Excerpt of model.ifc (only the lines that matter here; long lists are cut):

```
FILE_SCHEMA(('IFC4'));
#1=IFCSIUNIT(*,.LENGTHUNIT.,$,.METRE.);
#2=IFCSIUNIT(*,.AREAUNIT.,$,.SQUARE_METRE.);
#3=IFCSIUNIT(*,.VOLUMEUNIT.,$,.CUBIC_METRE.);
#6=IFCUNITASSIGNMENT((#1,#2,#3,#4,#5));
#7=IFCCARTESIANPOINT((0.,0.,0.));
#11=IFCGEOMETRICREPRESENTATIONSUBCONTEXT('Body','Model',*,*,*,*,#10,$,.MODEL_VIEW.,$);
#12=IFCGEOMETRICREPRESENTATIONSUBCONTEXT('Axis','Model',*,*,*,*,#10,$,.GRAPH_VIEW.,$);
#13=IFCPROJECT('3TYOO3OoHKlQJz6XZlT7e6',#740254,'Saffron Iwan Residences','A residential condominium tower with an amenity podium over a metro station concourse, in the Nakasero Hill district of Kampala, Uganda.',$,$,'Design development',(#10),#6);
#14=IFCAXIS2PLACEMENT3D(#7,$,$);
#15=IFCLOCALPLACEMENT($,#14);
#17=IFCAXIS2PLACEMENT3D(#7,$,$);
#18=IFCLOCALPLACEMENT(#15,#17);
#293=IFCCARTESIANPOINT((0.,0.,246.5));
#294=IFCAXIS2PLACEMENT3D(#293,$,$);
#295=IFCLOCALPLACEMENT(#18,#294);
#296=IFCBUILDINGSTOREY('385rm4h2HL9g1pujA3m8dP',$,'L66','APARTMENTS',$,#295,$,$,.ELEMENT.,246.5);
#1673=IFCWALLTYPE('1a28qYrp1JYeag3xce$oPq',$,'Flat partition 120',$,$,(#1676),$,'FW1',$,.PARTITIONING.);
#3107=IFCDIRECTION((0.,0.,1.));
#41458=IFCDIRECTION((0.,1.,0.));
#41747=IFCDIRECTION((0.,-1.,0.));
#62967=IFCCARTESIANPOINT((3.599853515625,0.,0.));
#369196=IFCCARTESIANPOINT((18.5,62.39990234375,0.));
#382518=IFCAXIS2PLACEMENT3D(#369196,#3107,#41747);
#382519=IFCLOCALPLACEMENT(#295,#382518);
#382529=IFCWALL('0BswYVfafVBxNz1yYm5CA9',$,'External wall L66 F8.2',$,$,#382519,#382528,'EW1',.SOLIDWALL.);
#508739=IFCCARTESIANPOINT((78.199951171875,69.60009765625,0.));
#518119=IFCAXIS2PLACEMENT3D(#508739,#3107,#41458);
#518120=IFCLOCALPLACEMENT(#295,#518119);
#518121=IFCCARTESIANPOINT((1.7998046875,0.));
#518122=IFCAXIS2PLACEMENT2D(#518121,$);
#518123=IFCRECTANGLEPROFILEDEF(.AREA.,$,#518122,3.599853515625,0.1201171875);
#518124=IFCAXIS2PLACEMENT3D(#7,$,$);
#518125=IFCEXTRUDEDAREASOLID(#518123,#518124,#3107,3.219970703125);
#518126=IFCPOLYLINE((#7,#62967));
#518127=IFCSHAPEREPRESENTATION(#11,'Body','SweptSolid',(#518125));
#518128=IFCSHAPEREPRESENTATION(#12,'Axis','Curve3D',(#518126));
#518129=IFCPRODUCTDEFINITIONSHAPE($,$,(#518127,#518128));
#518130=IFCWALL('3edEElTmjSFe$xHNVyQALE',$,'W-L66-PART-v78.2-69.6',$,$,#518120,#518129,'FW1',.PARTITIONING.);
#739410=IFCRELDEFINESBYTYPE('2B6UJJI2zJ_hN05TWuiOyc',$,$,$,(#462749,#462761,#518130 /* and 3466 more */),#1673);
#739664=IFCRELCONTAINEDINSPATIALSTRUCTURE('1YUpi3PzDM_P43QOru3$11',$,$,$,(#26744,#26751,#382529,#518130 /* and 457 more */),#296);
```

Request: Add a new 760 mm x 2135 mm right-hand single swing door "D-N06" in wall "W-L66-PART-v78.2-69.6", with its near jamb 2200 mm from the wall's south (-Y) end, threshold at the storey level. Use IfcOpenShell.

```python
import numpy as np
import ifcopenshell
import ifcopenshell.api.feature
import ifcopenshell.api.geometry
import ifcopenshell.api.root
import ifcopenshell.api.spatial
import ifcopenshell.geom
import ifcopenshell.util.element
import ifcopenshell.util.placement
import ifcopenshell.util.representation
import ifcopenshell.util.shape
import ifcopenshell.util.unit

model = ifcopenshell.open("model.ifc")
unit_scale = ifcopenshell.util.unit.calculate_unit_scale(model)
settings = ifcopenshell.geom.settings()


def volume(element):
    """Net volume in cubic metres, openings subtracted."""
    shape = ifcopenshell.geom.create_shape(settings, element)
    return ifcopenshell.util.shape.get_volume(shape.geometry)


wall = model.by_guid("3edEElTmjSFe$xHNVyQALE")
storey = ifcopenshell.util.element.get_container(wall, ifc_class="IfcBuildingStorey")
context = ifcopenshell.util.representation.get_context(model, "Model", "Body", "MODEL_VIEW")
before = volume(wall)

width, height, from_end, sill = 0.76, 2.135, 2.2, 0.0  # metres

# The wall runs along its own X axis, and the end named is its -X end.
wall_shape = ifcopenshell.geom.create_shape(settings, wall)
x, y, z = ifcopenshell.util.shape.get_vertices(wall_shape.geometry).T
start = x.min() + from_end
face, thickness = float(y.min()), float(y.max() - y.min())
wall_matrix = ifcopenshell.util.placement.get_local_placement(wall.ObjectPlacement)
level = ifcopenshell.util.placement.get_local_placement(storey.ObjectPlacement)[2, 3]


def in_wall(x, y):
    """Placement at x, y metres in the wall's axes, at sill height."""
    matrix = wall_matrix.copy()
    matrix[:, 3] = wall_matrix @ np.array([x / unit_scale, y / unit_scale, 0.0, 1.0])
    matrix[2, 3] = level + sill / unit_scale
    return matrix


# Opening: a box that overshoots both wall faces by 50 mm.
opening = ifcopenshell.api.root.create_entity(model, ifc_class="IfcOpeningElement", predefined_type="OPENING")
box = ifcopenshell.api.geometry.add_wall_representation(
    model, context=context, length=width, height=height, thickness=thickness + 0.1
)
ifcopenshell.api.geometry.assign_representation(model, product=opening, representation=box)
ifcopenshell.api.geometry.edit_object_placement(model, product=opening, matrix=in_wall(start, face - 0.05), is_si=False)
ifcopenshell.api.feature.add_feature(model, feature=opening, element=wall)

door = ifcopenshell.api.root.create_entity(model, ifc_class="IfcDoor", name="D-N06", predefined_type="DOOR")
door.OverallWidth, door.OverallHeight = width / unit_scale, height / unit_scale
door.OperationType = "SINGLE_SWING_RIGHT"
body = ifcopenshell.api.geometry.add_door_representation(
    model,
    context=context,
    overall_width=door.OverallWidth,
    overall_height=door.OverallHeight,
    operation_type="SINGLE_SWING_RIGHT",
    lining_properties={"LiningDepth": thickness / unit_scale, "ThresholdDepth": thickness / unit_scale},
)
ifcopenshell.api.geometry.assign_representation(model, product=door, representation=body)
ifcopenshell.api.spatial.assign_container(model, products=[door], relating_structure=storey)
ifcopenshell.api.feature.add_filling(model, opening=opening, element=door)

# The lining spans the wall, so the door starts at the wall face.
ifcopenshell.api.geometry.edit_object_placement(model, product=door, matrix=in_wall(start, face), is_si=False)

after = volume(wall)

print(f"wall volume {before:.3f} -> {after:.3f} m3")

model.write("model_updated.ifc")
```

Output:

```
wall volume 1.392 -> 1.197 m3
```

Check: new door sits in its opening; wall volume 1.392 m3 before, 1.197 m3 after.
